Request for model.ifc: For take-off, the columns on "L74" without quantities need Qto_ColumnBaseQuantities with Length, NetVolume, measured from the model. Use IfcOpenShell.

First a look at what the model holds.

```python
import ifcopenshell
import ifcopenshell.util.element
import ifcopenshell.util.unit

model = ifcopenshell.open("model.ifc")
print(model.schema)
for unit_type in ("LENGTHUNIT", "AREAUNIT", "VOLUMEUNIT"):
    print(unit_type, ifcopenshell.util.unit.calculate_unit_scale(model, unit_type))
storey = next(s for s in model.by_type("IfcBuildingStorey") if s.Name == "L74")
columns = [e for e in ifcopenshell.util.element.get_decomposition(storey) if e.is_a("IfcColumn")]
for e in sorted(columns, key=lambda e: e.id()):
    print(e.id(), e.is_a(), e.Name, list(ifcopenshell.util.element.get_psets(e, qtos_only=True)), sep=" | ")
```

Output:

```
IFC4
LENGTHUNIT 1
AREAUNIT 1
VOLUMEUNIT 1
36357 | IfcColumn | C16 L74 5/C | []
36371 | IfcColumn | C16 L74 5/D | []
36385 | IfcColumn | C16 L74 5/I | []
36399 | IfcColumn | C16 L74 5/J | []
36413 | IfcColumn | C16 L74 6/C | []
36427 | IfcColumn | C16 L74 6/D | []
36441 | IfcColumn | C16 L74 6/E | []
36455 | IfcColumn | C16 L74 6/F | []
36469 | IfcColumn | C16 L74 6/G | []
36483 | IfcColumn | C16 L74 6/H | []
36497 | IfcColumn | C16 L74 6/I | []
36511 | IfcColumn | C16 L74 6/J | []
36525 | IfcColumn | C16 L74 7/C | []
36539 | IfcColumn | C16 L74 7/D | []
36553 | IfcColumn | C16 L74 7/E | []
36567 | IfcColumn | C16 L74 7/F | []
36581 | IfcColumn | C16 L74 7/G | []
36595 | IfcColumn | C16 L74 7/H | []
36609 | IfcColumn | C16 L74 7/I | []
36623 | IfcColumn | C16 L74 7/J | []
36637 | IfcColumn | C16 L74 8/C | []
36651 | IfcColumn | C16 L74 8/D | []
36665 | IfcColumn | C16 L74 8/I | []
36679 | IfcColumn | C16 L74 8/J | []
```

```python
import ifcopenshell
import ifcopenshell.api.pset
import ifcopenshell.geom
import ifcopenshell.util.element
import ifcopenshell.util.shape
import ifcopenshell.util.unit

model = ifcopenshell.open("model.ifc")
unit_scale = ifcopenshell.util.unit.calculate_unit_scale(model)
volume_scale = ifcopenshell.util.unit.calculate_unit_scale(model, "VOLUMEUNIT")
settings = ifcopenshell.geom.settings()

storey = next(s for s in model.by_type("IfcBuildingStorey") if s.Name == "L74")
columns = [e for e in ifcopenshell.util.element.get_decomposition(storey) if e.is_a("IfcColumn")]

for e in sorted(columns, key=lambda e: e.id()):
    if ifcopenshell.util.element.get_psets(e, qtos_only=True, should_inherit=False):
        continue
    # Geometry comes back in metres, in the element's own axes.
    shape = ifcopenshell.geom.create_shape(settings, e)
    values = {
        "Length": ifcopenshell.util.shape.get_z(shape.geometry) / unit_scale,
        "NetVolume": ifcopenshell.util.shape.get_volume(shape.geometry) / volume_scale,
    }
    qto = ifcopenshell.api.pset.add_qto(model, product=e, name="Qto_ColumnBaseQuantities")
    ifcopenshell.api.pset.edit_qto(model, qto=qto, properties=values)
    print(e.id(), {k: round(v, 3) for k, v in values.items()})

model.write("model_updated.ifc")
```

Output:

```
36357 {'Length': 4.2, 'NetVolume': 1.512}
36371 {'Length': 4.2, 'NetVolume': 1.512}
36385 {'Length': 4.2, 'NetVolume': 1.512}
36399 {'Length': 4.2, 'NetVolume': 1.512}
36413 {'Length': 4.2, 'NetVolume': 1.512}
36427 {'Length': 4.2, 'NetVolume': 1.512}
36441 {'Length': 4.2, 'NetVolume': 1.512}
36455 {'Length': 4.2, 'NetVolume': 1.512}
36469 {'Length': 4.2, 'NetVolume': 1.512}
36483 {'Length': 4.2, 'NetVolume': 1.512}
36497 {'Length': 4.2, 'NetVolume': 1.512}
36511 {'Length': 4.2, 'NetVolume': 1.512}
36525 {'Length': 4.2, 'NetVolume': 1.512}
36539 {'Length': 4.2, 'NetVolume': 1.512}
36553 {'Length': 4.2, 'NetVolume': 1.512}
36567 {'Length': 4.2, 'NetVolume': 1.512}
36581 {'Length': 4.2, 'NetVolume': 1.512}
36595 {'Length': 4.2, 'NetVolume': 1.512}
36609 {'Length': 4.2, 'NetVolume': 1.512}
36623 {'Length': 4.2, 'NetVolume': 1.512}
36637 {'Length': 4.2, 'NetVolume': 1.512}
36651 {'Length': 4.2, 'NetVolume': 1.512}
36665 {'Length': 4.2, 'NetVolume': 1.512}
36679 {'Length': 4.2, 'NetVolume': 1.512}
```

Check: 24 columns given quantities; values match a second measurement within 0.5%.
